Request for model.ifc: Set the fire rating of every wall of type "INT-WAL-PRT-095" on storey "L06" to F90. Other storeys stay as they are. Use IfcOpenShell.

First a look at what the model holds.

```python
import ifcopenshell
import ifcopenshell.util.element

model = ifcopenshell.open("model.ifc")
print(model.schema)
storey = next(s for s in model.by_type("IfcBuildingStorey") if s.Name == "L06")
walls = [e for e in ifcopenshell.util.element.get_decomposition(storey) if e.is_a("IfcWall")]
seen = {}
for e in walls:
    element_type = ifcopenshell.util.element.get_type(e)
    key = (element_type.Name if element_type != e and element_type else None, ifcopenshell.util.element.get_pset(e, "Pset_WallCommon", "FireRating"))
    seen[key] = seen.get(key, 0) + 1
for (name, value), count in sorted(seen.items(), key=str):
    print(count, "x", name, "|", value)
```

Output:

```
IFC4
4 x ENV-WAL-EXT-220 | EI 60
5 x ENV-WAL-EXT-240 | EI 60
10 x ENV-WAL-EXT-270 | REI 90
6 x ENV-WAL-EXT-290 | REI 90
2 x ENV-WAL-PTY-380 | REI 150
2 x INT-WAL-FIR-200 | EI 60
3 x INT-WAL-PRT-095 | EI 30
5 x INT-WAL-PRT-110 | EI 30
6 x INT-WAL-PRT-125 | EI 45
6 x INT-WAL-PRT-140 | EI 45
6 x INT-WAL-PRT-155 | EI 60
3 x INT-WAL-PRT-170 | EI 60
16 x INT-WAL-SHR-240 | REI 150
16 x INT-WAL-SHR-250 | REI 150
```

```python
import ifcopenshell
import ifcopenshell.api.pset
import ifcopenshell.util.element

model = ifcopenshell.open("model.ifc")

storey = next(s for s in model.by_type("IfcBuildingStorey") if s.Name == "L06")
walls = [e for e in ifcopenshell.util.element.get_decomposition(storey) if e.is_a("IfcWall")]

count = 0
for e in walls:
    element_type = ifcopenshell.util.element.get_type(e)
    if element_type in (None, e) or element_type.Name != "INT-WAL-PRT-095":
        continue
    # add_pset returns the element's existing set when there is one.
    pset = ifcopenshell.api.pset.add_pset(model, product=e, name="Pset_WallCommon")
    ifcopenshell.api.pset.edit_pset(model, pset=pset, properties={"FireRating": "F90"})
    count += 1

print(count, "walls updated")

model.write("model_updated.ifc")
```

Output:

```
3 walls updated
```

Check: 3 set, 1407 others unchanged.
